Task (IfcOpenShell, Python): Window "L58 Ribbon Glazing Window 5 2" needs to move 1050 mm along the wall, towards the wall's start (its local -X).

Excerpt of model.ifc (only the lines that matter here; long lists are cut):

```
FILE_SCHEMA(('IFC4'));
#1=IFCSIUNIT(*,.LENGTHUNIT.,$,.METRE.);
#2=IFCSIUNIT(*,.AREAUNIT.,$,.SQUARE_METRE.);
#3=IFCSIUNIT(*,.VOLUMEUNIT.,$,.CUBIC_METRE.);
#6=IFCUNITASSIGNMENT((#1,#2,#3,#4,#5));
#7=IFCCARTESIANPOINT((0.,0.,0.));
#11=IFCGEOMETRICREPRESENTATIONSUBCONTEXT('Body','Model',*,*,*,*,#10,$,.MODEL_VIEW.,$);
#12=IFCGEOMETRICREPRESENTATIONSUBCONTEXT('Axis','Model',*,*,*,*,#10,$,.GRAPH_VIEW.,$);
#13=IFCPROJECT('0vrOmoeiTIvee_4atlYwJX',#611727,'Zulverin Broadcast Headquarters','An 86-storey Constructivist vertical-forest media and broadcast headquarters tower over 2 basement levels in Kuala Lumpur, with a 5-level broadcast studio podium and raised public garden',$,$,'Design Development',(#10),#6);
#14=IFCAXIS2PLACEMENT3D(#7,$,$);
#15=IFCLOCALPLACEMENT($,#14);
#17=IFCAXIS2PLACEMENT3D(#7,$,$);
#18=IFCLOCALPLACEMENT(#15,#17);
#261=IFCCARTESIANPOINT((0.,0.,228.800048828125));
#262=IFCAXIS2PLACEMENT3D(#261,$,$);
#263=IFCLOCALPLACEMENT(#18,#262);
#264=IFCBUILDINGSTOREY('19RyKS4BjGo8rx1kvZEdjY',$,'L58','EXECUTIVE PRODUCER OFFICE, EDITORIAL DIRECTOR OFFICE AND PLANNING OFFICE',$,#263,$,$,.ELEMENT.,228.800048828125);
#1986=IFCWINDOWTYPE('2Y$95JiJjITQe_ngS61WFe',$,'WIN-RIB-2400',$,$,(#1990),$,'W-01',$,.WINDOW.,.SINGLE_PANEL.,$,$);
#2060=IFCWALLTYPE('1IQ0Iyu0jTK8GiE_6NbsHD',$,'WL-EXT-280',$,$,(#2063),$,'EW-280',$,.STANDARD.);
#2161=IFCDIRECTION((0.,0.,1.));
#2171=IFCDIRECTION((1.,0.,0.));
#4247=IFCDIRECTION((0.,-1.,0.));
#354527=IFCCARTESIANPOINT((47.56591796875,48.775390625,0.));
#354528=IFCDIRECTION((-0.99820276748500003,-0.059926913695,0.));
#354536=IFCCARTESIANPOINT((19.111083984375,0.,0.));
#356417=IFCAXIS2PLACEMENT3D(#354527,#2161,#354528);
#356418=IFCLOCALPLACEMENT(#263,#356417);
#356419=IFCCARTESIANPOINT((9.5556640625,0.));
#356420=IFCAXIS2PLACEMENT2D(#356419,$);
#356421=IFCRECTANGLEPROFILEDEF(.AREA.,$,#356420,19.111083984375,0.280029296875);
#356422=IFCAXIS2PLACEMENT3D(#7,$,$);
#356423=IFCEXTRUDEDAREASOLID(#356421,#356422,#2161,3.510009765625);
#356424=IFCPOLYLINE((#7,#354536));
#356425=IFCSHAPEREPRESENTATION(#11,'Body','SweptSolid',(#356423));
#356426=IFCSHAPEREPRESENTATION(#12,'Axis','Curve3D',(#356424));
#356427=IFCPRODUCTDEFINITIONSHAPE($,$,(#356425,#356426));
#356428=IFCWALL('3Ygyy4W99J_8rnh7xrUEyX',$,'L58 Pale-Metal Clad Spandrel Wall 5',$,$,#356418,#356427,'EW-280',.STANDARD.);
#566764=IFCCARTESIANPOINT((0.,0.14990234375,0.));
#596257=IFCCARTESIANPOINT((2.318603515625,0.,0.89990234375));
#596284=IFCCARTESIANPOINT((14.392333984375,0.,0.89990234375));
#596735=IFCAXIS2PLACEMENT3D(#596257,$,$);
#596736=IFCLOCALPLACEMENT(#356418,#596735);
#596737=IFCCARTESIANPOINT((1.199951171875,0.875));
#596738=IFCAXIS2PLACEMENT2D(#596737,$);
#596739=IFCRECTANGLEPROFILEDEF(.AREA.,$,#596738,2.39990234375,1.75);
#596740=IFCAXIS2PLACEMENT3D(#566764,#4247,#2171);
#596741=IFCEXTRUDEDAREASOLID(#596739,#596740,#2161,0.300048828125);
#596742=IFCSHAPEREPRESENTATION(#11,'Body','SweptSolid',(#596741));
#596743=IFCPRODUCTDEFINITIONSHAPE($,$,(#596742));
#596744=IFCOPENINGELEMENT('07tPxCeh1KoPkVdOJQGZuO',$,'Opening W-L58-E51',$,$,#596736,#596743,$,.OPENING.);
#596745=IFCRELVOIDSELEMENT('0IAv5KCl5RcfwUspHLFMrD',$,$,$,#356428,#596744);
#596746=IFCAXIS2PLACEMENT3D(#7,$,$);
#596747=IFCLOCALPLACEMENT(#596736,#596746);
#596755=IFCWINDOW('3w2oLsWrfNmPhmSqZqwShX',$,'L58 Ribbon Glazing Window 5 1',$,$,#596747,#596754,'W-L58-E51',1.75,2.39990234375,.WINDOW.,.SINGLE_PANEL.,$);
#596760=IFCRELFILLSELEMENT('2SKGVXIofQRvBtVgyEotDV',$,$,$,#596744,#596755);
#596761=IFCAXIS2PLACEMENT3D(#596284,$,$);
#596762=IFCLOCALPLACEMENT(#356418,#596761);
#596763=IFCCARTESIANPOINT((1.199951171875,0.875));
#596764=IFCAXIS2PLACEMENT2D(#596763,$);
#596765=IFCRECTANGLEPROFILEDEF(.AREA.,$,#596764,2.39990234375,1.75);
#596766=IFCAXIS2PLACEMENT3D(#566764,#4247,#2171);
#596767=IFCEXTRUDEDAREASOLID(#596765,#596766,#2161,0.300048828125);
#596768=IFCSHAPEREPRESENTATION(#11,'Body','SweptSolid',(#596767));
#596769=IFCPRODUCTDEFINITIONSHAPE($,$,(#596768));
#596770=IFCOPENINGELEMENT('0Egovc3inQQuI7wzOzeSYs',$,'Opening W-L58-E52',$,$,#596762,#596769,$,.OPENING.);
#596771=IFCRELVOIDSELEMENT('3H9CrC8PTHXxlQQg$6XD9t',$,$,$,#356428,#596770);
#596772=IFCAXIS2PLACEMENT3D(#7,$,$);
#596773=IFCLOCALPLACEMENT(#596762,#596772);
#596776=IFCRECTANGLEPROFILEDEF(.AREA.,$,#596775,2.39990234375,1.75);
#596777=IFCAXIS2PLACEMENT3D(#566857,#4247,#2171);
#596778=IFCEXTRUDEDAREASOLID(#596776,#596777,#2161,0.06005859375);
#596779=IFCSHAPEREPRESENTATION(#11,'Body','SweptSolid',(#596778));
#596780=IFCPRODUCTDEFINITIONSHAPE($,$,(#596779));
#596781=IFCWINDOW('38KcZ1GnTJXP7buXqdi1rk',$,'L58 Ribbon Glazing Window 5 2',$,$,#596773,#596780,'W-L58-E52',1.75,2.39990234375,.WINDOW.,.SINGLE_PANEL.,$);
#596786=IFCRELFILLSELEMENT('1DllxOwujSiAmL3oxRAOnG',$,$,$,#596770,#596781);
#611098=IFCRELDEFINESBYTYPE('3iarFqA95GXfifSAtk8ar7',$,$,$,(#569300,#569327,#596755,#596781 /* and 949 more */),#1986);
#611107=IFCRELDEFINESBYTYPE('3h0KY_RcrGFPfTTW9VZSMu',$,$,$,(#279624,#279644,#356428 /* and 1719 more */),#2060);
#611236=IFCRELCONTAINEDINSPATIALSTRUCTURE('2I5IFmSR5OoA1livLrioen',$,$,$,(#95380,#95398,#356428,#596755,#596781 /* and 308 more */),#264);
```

```python
import ifcopenshell
import ifcopenshell.api.geometry
import ifcopenshell.util.placement

model = ifcopenshell.open("model.ifc")

window = model.by_guid("38KcZ1GnTJXP7buXqdi1rk")
opening = window.FillsVoids[0].RelatingOpeningElement
wall = opening.VoidsElements[0].RelatingBuildingElement

wall_matrix = ifcopenshell.util.placement.get_local_placement(wall.ObjectPlacement)
shift = wall_matrix[:3, 0] * -1.05
before = ifcopenshell.util.placement.get_local_placement(window.ObjectPlacement)[:3, 3].copy()

# The window is placed relative to its opening, so it follows when the opening moves.
matrix = ifcopenshell.util.placement.get_local_placement(opening.ObjectPlacement)
matrix[:3, 3] += shift
ifcopenshell.api.geometry.edit_object_placement(
    model, product=opening, matrix=matrix, is_si=False, should_transform_children=True
)

after = ifcopenshell.util.placement.get_local_placement(window.ObjectPlacement)[:3, 3]
print("window moved by", (after - before).round(3) + 0.0)

model.write("model_v2.ifc")
```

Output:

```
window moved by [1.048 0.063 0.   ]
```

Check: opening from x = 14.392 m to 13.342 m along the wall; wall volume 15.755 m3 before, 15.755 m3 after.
